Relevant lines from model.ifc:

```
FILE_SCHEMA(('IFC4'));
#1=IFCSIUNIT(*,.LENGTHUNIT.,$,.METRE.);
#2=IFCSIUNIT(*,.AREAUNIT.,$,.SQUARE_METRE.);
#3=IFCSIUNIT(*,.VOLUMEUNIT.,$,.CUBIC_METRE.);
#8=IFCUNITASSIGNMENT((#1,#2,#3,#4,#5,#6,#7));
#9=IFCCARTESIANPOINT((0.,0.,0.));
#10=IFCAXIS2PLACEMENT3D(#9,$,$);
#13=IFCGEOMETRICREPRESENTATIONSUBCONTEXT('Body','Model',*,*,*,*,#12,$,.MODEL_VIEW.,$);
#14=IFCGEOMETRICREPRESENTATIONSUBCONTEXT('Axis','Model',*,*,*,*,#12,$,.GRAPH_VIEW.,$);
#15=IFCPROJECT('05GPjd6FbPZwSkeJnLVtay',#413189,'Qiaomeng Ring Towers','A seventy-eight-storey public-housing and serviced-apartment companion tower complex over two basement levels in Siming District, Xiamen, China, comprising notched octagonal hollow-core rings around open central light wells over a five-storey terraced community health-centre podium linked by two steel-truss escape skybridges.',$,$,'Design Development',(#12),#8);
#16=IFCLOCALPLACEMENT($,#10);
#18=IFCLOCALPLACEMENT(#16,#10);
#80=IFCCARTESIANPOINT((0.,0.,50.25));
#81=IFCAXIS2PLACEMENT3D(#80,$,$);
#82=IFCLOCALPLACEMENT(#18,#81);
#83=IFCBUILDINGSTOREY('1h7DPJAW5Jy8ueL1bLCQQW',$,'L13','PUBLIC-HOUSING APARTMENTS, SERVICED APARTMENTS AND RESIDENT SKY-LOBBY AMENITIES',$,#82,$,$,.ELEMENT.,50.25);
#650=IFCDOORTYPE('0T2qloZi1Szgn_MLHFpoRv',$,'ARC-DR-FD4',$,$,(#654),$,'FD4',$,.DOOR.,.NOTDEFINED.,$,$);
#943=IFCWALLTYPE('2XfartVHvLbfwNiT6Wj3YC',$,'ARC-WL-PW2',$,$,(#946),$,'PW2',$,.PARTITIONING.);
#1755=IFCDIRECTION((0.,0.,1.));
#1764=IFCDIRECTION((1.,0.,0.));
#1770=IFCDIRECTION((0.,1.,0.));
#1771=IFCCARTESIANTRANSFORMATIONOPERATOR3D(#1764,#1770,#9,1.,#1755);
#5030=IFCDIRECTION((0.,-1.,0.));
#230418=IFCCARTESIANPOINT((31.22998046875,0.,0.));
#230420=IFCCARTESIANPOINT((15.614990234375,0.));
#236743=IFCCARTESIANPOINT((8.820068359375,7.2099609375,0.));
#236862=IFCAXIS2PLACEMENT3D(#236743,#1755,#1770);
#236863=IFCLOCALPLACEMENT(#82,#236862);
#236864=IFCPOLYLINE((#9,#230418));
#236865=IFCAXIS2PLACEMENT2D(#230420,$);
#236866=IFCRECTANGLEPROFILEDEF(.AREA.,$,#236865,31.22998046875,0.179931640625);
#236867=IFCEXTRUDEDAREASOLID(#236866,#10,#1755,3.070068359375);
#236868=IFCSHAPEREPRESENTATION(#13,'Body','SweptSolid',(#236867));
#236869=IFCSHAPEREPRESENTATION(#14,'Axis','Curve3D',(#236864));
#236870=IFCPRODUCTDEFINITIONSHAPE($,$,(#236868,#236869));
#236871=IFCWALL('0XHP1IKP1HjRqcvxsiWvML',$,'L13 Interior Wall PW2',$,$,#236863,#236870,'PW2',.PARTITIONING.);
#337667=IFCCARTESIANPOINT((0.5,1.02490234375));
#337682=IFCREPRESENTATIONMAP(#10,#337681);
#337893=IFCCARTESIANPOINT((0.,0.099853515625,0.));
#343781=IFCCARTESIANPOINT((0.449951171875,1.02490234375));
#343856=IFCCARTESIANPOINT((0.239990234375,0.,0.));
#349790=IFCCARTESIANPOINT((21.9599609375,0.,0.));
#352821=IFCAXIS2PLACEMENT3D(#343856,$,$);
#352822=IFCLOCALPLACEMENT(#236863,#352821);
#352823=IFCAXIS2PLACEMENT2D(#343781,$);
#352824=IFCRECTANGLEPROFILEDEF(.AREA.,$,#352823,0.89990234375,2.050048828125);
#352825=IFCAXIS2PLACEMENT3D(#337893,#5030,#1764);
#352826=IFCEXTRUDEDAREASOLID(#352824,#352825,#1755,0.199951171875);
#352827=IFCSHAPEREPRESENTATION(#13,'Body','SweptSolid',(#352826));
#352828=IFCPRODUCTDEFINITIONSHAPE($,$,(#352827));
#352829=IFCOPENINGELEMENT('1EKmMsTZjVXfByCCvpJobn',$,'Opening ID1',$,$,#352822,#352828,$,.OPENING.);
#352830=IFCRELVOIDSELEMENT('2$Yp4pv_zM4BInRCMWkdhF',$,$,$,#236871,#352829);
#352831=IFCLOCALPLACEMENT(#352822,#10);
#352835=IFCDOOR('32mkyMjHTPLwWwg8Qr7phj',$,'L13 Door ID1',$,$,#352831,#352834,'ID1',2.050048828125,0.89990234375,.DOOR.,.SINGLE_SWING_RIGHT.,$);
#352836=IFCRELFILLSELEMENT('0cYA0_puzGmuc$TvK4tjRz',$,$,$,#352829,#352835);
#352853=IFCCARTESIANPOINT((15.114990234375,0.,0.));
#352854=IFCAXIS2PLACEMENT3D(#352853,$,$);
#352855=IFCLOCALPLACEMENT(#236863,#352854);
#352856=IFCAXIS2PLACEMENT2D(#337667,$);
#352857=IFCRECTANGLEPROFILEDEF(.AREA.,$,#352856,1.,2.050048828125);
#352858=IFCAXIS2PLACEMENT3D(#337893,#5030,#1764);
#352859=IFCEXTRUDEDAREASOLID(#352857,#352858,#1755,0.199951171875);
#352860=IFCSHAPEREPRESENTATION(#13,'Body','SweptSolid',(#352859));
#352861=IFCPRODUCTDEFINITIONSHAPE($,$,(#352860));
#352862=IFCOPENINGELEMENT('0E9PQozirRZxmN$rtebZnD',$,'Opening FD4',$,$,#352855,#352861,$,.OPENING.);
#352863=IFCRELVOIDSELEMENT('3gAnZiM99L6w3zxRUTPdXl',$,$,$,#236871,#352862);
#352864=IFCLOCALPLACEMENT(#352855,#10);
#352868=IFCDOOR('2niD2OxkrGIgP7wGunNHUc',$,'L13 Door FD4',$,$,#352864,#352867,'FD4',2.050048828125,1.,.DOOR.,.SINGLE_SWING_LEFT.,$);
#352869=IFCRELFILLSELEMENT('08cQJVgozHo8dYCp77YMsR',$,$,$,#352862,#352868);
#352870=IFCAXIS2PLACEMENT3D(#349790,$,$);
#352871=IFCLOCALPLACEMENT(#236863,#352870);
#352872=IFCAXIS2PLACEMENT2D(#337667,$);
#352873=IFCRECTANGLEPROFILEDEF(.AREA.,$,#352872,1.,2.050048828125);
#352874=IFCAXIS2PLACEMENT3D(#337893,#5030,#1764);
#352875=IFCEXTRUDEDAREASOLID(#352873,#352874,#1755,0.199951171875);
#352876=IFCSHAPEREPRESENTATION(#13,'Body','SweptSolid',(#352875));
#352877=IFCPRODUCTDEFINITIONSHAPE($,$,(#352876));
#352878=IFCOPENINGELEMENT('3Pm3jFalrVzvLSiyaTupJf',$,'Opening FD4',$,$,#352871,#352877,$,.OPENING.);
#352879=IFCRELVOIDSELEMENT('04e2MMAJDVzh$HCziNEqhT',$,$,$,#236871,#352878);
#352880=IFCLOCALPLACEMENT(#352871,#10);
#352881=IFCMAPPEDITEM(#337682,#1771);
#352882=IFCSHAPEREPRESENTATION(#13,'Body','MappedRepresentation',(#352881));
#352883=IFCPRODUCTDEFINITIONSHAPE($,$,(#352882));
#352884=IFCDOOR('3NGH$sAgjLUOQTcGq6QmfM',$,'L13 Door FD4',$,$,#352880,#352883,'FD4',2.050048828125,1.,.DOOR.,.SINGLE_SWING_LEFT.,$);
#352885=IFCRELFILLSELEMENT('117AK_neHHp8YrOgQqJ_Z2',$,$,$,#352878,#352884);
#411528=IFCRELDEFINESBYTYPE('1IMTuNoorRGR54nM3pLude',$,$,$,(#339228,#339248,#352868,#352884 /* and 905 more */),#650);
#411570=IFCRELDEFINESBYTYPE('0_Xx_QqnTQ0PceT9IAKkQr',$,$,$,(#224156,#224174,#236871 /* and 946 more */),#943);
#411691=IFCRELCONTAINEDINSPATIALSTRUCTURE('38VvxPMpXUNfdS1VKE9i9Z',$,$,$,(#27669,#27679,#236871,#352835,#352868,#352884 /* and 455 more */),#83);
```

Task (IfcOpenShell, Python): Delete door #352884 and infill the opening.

```python
import ifcopenshell
import ifcopenshell.api.feature
import ifcopenshell.api.root
import ifcopenshell.geom
import ifcopenshell.util.shape

model = ifcopenshell.open("model.ifc")
settings = ifcopenshell.geom.settings()


def volume(element):
    """Net volume in cubic metres, openings subtracted."""
    shape = ifcopenshell.geom.create_shape(settings, element)
    return ifcopenshell.util.shape.get_volume(shape.geometry)


door = model.by_guid("3NGH$sAgjLUOQTcGq6QmfM")
opening = door.FillsVoids[0].RelatingOpeningElement
wall = opening.VoidsElements[0].RelatingBuildingElement
before = volume(wall)

ifcopenshell.api.root.remove_product(model, product=door)
ifcopenshell.api.feature.remove_feature(model, feature=opening)

after = volume(wall)

print(f"wall volume {before:.3f} -> {after:.3f} m3")

model.write("model_edited.ifc")
```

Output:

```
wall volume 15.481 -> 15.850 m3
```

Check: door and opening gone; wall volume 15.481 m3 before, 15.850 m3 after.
